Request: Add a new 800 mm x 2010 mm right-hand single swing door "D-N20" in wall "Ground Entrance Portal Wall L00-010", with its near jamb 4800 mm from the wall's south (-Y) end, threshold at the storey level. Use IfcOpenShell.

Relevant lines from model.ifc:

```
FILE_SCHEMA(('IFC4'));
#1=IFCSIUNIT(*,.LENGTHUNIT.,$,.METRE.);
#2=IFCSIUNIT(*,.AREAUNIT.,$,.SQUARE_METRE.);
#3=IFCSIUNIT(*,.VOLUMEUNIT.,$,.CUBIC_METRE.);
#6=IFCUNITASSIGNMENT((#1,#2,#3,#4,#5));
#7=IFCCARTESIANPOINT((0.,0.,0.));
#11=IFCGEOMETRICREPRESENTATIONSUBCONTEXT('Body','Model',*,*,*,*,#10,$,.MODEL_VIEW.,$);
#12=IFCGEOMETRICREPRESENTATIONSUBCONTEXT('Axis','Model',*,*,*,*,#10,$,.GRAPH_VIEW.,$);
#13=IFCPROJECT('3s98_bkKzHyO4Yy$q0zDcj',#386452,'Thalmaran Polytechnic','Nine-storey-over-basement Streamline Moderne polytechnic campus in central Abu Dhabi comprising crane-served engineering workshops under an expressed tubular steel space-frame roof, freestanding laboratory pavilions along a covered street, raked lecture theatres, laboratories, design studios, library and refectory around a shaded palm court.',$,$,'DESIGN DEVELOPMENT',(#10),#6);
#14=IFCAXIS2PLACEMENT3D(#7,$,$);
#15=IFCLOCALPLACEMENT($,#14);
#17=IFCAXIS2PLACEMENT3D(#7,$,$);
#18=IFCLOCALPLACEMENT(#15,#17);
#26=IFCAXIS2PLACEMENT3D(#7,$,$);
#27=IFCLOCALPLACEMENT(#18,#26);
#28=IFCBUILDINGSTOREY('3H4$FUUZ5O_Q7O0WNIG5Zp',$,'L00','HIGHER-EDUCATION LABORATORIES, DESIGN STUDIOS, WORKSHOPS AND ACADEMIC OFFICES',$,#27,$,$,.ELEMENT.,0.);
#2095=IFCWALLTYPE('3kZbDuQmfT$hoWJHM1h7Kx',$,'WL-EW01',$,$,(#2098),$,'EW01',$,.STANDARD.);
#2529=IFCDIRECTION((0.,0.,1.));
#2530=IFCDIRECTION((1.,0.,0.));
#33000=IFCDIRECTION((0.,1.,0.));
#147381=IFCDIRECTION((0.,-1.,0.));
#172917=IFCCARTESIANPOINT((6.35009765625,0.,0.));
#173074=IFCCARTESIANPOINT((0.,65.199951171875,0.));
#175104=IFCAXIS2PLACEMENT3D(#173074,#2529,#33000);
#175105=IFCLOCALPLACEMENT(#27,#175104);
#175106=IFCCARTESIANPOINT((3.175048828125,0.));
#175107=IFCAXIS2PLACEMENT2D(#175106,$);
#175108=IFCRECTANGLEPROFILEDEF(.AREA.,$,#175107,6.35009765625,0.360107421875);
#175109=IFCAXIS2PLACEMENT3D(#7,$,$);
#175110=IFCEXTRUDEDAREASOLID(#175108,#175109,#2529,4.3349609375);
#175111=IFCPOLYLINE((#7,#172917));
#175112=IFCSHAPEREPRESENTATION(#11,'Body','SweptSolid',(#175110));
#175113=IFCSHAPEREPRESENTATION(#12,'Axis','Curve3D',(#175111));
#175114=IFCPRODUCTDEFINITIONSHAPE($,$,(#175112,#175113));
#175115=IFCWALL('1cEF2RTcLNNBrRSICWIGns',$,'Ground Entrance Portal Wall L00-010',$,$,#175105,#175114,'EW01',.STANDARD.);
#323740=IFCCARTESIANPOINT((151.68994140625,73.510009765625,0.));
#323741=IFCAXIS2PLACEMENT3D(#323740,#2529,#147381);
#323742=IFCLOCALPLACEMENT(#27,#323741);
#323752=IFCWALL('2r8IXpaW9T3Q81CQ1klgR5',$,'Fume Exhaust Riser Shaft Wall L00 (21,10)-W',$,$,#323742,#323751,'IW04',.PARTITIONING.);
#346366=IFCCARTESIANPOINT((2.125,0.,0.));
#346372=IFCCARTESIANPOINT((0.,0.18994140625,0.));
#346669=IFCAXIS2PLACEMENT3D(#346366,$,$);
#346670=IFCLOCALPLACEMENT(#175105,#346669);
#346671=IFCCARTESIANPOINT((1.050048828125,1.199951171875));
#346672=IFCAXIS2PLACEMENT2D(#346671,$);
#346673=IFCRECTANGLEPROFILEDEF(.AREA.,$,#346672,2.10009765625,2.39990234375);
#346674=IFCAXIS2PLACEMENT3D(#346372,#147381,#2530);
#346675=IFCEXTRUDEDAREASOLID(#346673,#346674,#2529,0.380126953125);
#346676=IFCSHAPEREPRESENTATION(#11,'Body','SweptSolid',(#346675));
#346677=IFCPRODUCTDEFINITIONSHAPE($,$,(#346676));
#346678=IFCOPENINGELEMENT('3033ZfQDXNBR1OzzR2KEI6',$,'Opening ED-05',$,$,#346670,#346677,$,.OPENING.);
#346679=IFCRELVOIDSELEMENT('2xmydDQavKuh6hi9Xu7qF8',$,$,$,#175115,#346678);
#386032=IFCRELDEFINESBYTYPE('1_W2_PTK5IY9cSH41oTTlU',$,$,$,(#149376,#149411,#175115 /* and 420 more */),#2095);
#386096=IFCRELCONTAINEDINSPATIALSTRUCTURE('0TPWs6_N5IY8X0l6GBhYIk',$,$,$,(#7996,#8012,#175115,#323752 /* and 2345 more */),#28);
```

```python
import numpy as np
import ifcopenshell
import ifcopenshell.api.feature
import ifcopenshell.api.geometry
import ifcopenshell.api.root
import ifcopenshell.api.spatial
import ifcopenshell.geom
import ifcopenshell.util.element
import ifcopenshell.util.placement
import ifcopenshell.util.representation
import ifcopenshell.util.shape
import ifcopenshell.util.unit

model = ifcopenshell.open("model.ifc")
unit_scale = ifcopenshell.util.unit.calculate_unit_scale(model)
settings = ifcopenshell.geom.settings()


def volume(element):
    """Net volume in cubic metres, openings subtracted."""
    shape = ifcopenshell.geom.create_shape(settings, element)
    return ifcopenshell.util.shape.get_volume(shape.geometry)


wall = model.by_guid("1cEF2RTcLNNBrRSICWIGns")
storey = ifcopenshell.util.element.get_container(wall, ifc_class="IfcBuildingStorey")
context = ifcopenshell.util.representation.get_context(model, "Model", "Body", "MODEL_VIEW")
before = volume(wall)

width, height, from_end, sill = 0.8, 2.01, 4.8, 0.0  # metres

# The wall runs along its own X axis, and the end named is its -X end.
wall_shape = ifcopenshell.geom.create_shape(settings, wall)
x, y, z = ifcopenshell.util.shape.get_vertices(wall_shape.geometry).T
start = x.min() + from_end
face, thickness = float(y.min()), float(y.max() - y.min())
wall_matrix = ifcopenshell.util.placement.get_local_placement(wall.ObjectPlacement)
level = ifcopenshell.util.placement.get_local_placement(storey.ObjectPlacement)[2, 3]


def in_wall(x, y):
    """Placement at x, y metres in the wall's axes, at sill height."""
    matrix = wall_matrix.copy()
    matrix[:, 3] = wall_matrix @ np.array([x / unit_scale, y / unit_scale, 0.0, 1.0])
    matrix[2, 3] = level + sill / unit_scale
    return matrix


# Opening: a box that overshoots both wall faces by 50 mm.
opening = ifcopenshell.api.root.create_entity(model, ifc_class="IfcOpeningElement", predefined_type="OPENING")
box = ifcopenshell.api.geometry.add_wall_representation(
    model, context=context, length=width, height=height, thickness=thickness + 0.1
)
ifcopenshell.api.geometry.assign_representation(model, product=opening, representation=box)
ifcopenshell.api.geometry.edit_object_placement(model, product=opening, matrix=in_wall(start, face - 0.05), is_si=False)
ifcopenshell.api.feature.add_feature(model, feature=opening, element=wall)

door = ifcopenshell.api.root.create_entity(model, ifc_class="IfcDoor", name="D-N20", predefined_type="DOOR")
door.OverallWidth, door.OverallHeight = width / unit_scale, height / unit_scale
door.OperationType = "SINGLE_SWING_RIGHT"
body = ifcopenshell.api.geometry.add_door_representation(
    model,
    context=context,
    overall_width=door.OverallWidth,
    overall_height=door.OverallHeight,
    operation_type="SINGLE_SWING_RIGHT",
    lining_properties={"LiningDepth": thickness / unit_scale, "ThresholdDepth": thickness / unit_scale},
)
ifcopenshell.api.geometry.assign_representation(model, product=door, representation=body)
ifcopenshell.api.spatial.assign_container(model, products=[door], relating_structure=storey)
ifcopenshell.api.feature.add_filling(model, opening=opening, element=door)

# The lining spans the wall, so the door starts at the wall face.
ifcopenshell.api.geometry.edit_object_placement(model, product=door, matrix=in_wall(start, face), is_si=False)

after = volume(wall)

print(f"wall volume {before:.3f} -> {after:.3f} m3")

model.write("model_v2.ifc")
```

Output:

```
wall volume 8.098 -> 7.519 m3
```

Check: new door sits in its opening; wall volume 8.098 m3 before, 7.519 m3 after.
